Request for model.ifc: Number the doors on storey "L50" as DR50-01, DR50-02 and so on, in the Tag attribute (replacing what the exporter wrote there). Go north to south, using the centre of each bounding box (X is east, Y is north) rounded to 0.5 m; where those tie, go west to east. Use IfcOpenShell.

First a look at what the model holds.

```python
import ifcopenshell
import ifcopenshell.util.element
import ifcopenshell.util.placement

model = ifcopenshell.open("model.ifc")
print(model.schema)
storey = next(s for s in model.by_type("IfcBuildingStorey") if s.Name == "L50")
doors = [e for e in ifcopenshell.util.element.get_decomposition(storey) if e.is_a("IfcDoor")]
for e in sorted(doors, key=lambda e: e.id()):
    origin = ifcopenshell.util.placement.get_local_placement(e.ObjectPlacement)[:3, 3]
    print(e.id(), e.Tag, e.Name, origin.round(2) + 0.0, sep=" | ")
```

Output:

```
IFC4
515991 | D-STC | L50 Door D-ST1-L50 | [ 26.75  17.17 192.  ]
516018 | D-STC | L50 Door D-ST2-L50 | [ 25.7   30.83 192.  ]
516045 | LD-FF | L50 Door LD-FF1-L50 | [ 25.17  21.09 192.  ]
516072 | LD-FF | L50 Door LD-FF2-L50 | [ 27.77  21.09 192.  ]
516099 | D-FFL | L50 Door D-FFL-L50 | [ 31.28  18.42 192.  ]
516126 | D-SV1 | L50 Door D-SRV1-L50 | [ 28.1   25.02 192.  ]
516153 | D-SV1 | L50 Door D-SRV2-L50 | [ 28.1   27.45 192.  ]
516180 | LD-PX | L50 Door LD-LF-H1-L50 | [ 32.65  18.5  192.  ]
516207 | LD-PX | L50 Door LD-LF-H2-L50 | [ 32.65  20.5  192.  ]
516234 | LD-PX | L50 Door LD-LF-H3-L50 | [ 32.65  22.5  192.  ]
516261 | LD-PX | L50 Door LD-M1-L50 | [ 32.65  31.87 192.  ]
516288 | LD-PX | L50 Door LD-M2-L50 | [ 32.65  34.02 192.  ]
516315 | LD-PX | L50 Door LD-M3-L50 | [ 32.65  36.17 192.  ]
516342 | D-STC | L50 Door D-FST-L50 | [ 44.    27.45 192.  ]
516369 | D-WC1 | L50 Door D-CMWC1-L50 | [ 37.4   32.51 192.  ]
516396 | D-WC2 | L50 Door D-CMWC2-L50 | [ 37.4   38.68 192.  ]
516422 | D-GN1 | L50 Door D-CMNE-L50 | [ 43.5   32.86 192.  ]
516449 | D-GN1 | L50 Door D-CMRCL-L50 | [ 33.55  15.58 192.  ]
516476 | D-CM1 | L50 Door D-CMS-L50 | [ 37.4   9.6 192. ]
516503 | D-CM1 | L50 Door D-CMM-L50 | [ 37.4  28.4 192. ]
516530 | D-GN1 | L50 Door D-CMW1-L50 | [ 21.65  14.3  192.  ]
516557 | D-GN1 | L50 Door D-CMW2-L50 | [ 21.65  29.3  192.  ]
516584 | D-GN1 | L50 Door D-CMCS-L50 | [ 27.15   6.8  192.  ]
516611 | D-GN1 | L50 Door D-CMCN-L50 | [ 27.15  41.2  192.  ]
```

```python
import ifcopenshell
import ifcopenshell.geom
import ifcopenshell.util.element
import ifcopenshell.util.shape

model = ifcopenshell.open("model.ifc")
settings = ifcopenshell.geom.settings()
settings.set("use-world-coords", True)


def centre(element):
    shape = ifcopenshell.geom.create_shape(settings, element)
    return ifcopenshell.util.shape.get_bbox_centroid(shape.geometry)


storey = next(s for s in model.by_type("IfcBuildingStorey") if s.Name == "L50")
doors = [e for e in ifcopenshell.util.element.get_decomposition(storey) if e.is_a("IfcDoor")]

# Insertion points can sit at a corner or the storey origin, so sort by the geometry (in metres).
centres = {e: centre(e) for e in doors}
doors.sort(key=lambda e: (-round(centres[e][1] / 0.5), centres[e][0]))

for i, e in enumerate(doors, start=1):
    number = f"DR50-{i:02d}"
    e.Tag = number
    print(e.id(), number)

model.write("model_updated.ifc")
```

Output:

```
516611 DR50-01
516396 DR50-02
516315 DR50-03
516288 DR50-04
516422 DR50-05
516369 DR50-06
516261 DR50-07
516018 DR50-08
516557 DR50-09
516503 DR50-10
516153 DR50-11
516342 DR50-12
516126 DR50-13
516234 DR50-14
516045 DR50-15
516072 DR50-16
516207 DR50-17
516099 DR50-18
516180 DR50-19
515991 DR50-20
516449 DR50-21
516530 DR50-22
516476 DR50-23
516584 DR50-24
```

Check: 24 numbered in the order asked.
